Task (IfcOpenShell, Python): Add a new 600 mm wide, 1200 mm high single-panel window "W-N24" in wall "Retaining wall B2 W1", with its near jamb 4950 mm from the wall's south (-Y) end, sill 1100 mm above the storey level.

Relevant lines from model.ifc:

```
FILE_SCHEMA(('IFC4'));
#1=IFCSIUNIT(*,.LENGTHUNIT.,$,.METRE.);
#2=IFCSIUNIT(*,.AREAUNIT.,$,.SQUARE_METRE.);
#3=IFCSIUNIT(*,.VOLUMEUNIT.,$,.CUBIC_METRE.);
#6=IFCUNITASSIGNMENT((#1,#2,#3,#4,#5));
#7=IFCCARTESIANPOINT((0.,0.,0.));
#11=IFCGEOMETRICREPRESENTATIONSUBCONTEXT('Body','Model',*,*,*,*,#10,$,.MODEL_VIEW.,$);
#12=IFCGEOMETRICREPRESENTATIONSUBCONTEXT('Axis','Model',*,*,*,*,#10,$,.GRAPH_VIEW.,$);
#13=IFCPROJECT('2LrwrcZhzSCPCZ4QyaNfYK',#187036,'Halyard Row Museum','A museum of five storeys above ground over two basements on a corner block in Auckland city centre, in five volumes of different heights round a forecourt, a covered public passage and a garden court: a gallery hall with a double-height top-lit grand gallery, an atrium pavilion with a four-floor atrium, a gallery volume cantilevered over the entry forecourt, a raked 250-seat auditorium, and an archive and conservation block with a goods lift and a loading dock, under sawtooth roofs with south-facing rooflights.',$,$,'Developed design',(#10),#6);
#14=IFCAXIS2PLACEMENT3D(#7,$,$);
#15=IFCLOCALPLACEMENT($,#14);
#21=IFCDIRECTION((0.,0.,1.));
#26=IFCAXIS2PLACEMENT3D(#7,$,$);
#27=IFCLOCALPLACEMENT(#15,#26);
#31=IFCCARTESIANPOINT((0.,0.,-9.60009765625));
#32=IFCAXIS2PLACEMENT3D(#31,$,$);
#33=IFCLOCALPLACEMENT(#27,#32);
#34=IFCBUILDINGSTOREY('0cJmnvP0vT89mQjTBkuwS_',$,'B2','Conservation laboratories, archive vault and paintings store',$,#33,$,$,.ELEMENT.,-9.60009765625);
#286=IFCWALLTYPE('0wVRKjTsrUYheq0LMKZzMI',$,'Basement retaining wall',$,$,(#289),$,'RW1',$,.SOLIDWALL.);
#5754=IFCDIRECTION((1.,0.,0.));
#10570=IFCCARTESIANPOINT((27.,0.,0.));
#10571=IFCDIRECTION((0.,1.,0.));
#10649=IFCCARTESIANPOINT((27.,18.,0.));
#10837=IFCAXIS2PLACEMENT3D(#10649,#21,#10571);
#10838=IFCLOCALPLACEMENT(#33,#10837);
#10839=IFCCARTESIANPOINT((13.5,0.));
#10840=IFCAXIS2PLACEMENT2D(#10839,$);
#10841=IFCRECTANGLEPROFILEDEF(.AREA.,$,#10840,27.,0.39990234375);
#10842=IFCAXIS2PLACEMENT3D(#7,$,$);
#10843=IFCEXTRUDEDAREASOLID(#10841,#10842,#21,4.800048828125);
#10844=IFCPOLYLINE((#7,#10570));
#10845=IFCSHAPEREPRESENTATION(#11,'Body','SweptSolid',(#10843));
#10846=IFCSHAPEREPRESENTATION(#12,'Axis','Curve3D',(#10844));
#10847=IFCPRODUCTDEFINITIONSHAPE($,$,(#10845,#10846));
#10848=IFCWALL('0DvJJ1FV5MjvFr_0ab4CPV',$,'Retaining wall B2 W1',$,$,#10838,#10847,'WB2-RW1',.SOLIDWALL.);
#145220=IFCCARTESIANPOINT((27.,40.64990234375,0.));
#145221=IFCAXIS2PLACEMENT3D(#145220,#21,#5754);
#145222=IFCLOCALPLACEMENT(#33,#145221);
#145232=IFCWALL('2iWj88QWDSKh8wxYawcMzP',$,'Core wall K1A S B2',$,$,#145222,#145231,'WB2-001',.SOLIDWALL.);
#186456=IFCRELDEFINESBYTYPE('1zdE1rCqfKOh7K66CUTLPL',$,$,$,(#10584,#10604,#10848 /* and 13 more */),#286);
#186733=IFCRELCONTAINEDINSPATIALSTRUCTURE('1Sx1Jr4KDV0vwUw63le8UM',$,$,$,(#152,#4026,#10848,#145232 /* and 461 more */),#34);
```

```python
import numpy as np
import ifcopenshell
import ifcopenshell.api.feature
import ifcopenshell.api.geometry
import ifcopenshell.api.root
import ifcopenshell.api.spatial
import ifcopenshell.geom
import ifcopenshell.util.element
import ifcopenshell.util.placement
import ifcopenshell.util.representation
import ifcopenshell.util.shape
import ifcopenshell.util.unit

model = ifcopenshell.open("model.ifc")
unit_scale = ifcopenshell.util.unit.calculate_unit_scale(model)
settings = ifcopenshell.geom.settings()


def volume(element):
    """Net volume in cubic metres, openings subtracted."""
    shape = ifcopenshell.geom.create_shape(settings, element)
    return ifcopenshell.util.shape.get_volume(shape.geometry)


wall = model.by_guid("0DvJJ1FV5MjvFr_0ab4CPV")
storey = ifcopenshell.util.element.get_container(wall, ifc_class="IfcBuildingStorey")
context = ifcopenshell.util.representation.get_context(model, "Model", "Body", "MODEL_VIEW")
before = volume(wall)

width, height, from_end, sill = 0.6, 1.2, 4.95, 1.1  # metres

# The wall runs along its own X axis, and the end named is its -X end.
wall_shape = ifcopenshell.geom.create_shape(settings, wall)
x, y, z = ifcopenshell.util.shape.get_vertices(wall_shape.geometry).T
start = x.min() + from_end
face, thickness = float(y.min()), float(y.max() - y.min())
wall_matrix = ifcopenshell.util.placement.get_local_placement(wall.ObjectPlacement)
level = ifcopenshell.util.placement.get_local_placement(storey.ObjectPlacement)[2, 3]


def in_wall(x, y):
    """Placement at x, y metres in the wall's axes, at sill height."""
    matrix = wall_matrix.copy()
    matrix[:, 3] = wall_matrix @ np.array([x / unit_scale, y / unit_scale, 0.0, 1.0])
    matrix[2, 3] = level + sill / unit_scale
    return matrix


# Opening: a box that overshoots both wall faces by 50 mm.
opening = ifcopenshell.api.root.create_entity(model, ifc_class="IfcOpeningElement", predefined_type="OPENING")
box = ifcopenshell.api.geometry.add_wall_representation(
    model, context=context, length=width, height=height, thickness=thickness + 0.1
)
ifcopenshell.api.geometry.assign_representation(model, product=opening, representation=box)
ifcopenshell.api.geometry.edit_object_placement(model, product=opening, matrix=in_wall(start, face - 0.05), is_si=False)
ifcopenshell.api.feature.add_feature(model, feature=opening, element=wall)

window = ifcopenshell.api.root.create_entity(model, ifc_class="IfcWindow", name="W-N24", predefined_type="WINDOW")
window.OverallWidth, window.OverallHeight = width / unit_scale, height / unit_scale
window.PartitioningType = "SINGLE_PANEL"
body = ifcopenshell.api.geometry.add_window_representation(
    model,
    context=context,
    overall_width=window.OverallWidth,
    overall_height=window.OverallHeight,
    partition_type="SINGLE_PANEL",
)
ifcopenshell.api.geometry.assign_representation(model, product=window, representation=body)
ifcopenshell.api.spatial.assign_container(model, products=[window], relating_structure=storey)
ifcopenshell.api.feature.add_filling(model, opening=opening, element=window)

# Centre the window in the wall's thickness.
ifcopenshell.api.geometry.edit_object_placement(model, product=window, matrix=in_wall(start, face), is_si=False)
window_shape = ifcopenshell.geom.create_shape(settings, window)
depth = ifcopenshell.util.shape.get_vertices(window_shape.geometry)[:, 1]
offset = face + thickness / 2 - (depth.min() + depth.max()) / 2
ifcopenshell.api.geometry.edit_object_placement(model, product=window, matrix=in_wall(start, offset), is_si=False)

after = volume(wall)

print(f"wall volume {before:.3f} -> {after:.3f} m3")

model.write("model_updated.ifc")
```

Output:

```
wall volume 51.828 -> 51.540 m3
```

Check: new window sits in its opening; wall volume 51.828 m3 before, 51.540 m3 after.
